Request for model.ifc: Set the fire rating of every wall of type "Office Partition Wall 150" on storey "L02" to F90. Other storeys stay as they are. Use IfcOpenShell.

First a look at what the model holds.

```python
import ifcopenshell
import ifcopenshell.util.element

model = ifcopenshell.open("model.ifc")
print(model.schema)
storey = next(s for s in model.by_type("IfcBuildingStorey") if s.Name == "L02")
walls = [e for e in ifcopenshell.util.element.get_decomposition(storey) if e.is_a("IfcWall")]
seen = {}
for e in walls:
    element_type = ifcopenshell.util.element.get_type(e)
    key = (element_type.Name if element_type != e and element_type else None, ifcopenshell.util.element.get_pset(e, "Pset_WallCommon", "FireRating"))
    seen[key] = seen.get(key, 0) + 1
for (name, value), count in sorted(seen.items(), key=str):
    print(count, "x", name, "|", value)
```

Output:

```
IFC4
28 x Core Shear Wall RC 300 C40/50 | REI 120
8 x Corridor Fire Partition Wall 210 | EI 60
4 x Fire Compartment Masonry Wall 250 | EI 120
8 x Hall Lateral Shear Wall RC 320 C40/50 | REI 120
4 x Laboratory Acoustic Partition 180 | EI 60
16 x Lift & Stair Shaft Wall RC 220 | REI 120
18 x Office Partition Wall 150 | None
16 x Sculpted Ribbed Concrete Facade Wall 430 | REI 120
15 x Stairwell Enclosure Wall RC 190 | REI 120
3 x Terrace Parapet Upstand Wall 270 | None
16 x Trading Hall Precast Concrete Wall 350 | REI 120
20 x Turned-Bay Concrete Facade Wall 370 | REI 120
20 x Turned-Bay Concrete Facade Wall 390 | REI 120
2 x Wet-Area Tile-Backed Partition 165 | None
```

```python
import ifcopenshell
import ifcopenshell.api.pset
import ifcopenshell.util.element

model = ifcopenshell.open("model.ifc")

storey = next(s for s in model.by_type("IfcBuildingStorey") if s.Name == "L02")
walls = [e for e in ifcopenshell.util.element.get_decomposition(storey) if e.is_a("IfcWall")]

count = 0
for e in walls:
    element_type = ifcopenshell.util.element.get_type(e)
    if element_type in (None, e) or element_type.Name != "Office Partition Wall 150":
        continue
    # add_pset returns the element's existing set when there is one.
    pset = ifcopenshell.api.pset.add_pset(model, product=e, name="Pset_WallCommon")
    ifcopenshell.api.pset.edit_pset(model, pset=pset, properties={"FireRating": "F90"})
    count += 1

print(count, "walls updated")

model.write("model-out.ifc")
```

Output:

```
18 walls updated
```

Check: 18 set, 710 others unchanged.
